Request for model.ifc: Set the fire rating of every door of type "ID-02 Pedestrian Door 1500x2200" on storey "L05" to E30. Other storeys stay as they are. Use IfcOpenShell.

First a look at what the model holds.

```python
import ifcopenshell
import ifcopenshell.util.element

model = ifcopenshell.open("model.ifc")
print(model.schema)
storey = next(s for s in model.by_type("IfcBuildingStorey") if s.Name == "L05")
doors = [e for e in ifcopenshell.util.element.get_decomposition(storey) if e.is_a("IfcDoor")]
seen = {}
for e in doors:
    element_type = ifcopenshell.util.element.get_type(e)
    key = (element_type.Name if element_type != e and element_type else None, ifcopenshell.util.element.get_pset(e, "Pset_DoorCommon", "FireRating"))
    seen[key] = seen.get(key, 0) + 1
for (name, value), count in sorted(seen.items(), key=str):
    print(count, "x", name, "|", value)
```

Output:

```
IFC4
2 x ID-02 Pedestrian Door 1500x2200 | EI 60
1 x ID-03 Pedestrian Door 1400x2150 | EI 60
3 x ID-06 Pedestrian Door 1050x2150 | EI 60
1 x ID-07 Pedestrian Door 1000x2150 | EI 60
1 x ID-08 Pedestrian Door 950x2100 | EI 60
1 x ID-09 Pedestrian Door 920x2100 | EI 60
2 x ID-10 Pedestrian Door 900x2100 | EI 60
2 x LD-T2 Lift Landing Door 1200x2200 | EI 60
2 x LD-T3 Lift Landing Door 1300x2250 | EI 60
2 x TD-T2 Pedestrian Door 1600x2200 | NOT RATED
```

```python
import ifcopenshell
import ifcopenshell.api.pset
import ifcopenshell.util.element

model = ifcopenshell.open("model.ifc")

storey = next(s for s in model.by_type("IfcBuildingStorey") if s.Name == "L05")
doors = [e for e in ifcopenshell.util.element.get_decomposition(storey) if e.is_a("IfcDoor")]

count = 0
for e in doors:
    element_type = ifcopenshell.util.element.get_type(e)
    if element_type in (None, e) or element_type.Name != "ID-02 Pedestrian Door 1500x2200":
        continue
    # add_pset returns the element's existing set when there is one.
    pset = ifcopenshell.api.pset.add_pset(model, product=e, name="Pset_DoorCommon")
    ifcopenshell.api.pset.edit_pset(model, pset=pset, properties={"FireRating": "E30"})
    count += 1

print(count, "doors updated")

model.write("model_rev.ifc")
```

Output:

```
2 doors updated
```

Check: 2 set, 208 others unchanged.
